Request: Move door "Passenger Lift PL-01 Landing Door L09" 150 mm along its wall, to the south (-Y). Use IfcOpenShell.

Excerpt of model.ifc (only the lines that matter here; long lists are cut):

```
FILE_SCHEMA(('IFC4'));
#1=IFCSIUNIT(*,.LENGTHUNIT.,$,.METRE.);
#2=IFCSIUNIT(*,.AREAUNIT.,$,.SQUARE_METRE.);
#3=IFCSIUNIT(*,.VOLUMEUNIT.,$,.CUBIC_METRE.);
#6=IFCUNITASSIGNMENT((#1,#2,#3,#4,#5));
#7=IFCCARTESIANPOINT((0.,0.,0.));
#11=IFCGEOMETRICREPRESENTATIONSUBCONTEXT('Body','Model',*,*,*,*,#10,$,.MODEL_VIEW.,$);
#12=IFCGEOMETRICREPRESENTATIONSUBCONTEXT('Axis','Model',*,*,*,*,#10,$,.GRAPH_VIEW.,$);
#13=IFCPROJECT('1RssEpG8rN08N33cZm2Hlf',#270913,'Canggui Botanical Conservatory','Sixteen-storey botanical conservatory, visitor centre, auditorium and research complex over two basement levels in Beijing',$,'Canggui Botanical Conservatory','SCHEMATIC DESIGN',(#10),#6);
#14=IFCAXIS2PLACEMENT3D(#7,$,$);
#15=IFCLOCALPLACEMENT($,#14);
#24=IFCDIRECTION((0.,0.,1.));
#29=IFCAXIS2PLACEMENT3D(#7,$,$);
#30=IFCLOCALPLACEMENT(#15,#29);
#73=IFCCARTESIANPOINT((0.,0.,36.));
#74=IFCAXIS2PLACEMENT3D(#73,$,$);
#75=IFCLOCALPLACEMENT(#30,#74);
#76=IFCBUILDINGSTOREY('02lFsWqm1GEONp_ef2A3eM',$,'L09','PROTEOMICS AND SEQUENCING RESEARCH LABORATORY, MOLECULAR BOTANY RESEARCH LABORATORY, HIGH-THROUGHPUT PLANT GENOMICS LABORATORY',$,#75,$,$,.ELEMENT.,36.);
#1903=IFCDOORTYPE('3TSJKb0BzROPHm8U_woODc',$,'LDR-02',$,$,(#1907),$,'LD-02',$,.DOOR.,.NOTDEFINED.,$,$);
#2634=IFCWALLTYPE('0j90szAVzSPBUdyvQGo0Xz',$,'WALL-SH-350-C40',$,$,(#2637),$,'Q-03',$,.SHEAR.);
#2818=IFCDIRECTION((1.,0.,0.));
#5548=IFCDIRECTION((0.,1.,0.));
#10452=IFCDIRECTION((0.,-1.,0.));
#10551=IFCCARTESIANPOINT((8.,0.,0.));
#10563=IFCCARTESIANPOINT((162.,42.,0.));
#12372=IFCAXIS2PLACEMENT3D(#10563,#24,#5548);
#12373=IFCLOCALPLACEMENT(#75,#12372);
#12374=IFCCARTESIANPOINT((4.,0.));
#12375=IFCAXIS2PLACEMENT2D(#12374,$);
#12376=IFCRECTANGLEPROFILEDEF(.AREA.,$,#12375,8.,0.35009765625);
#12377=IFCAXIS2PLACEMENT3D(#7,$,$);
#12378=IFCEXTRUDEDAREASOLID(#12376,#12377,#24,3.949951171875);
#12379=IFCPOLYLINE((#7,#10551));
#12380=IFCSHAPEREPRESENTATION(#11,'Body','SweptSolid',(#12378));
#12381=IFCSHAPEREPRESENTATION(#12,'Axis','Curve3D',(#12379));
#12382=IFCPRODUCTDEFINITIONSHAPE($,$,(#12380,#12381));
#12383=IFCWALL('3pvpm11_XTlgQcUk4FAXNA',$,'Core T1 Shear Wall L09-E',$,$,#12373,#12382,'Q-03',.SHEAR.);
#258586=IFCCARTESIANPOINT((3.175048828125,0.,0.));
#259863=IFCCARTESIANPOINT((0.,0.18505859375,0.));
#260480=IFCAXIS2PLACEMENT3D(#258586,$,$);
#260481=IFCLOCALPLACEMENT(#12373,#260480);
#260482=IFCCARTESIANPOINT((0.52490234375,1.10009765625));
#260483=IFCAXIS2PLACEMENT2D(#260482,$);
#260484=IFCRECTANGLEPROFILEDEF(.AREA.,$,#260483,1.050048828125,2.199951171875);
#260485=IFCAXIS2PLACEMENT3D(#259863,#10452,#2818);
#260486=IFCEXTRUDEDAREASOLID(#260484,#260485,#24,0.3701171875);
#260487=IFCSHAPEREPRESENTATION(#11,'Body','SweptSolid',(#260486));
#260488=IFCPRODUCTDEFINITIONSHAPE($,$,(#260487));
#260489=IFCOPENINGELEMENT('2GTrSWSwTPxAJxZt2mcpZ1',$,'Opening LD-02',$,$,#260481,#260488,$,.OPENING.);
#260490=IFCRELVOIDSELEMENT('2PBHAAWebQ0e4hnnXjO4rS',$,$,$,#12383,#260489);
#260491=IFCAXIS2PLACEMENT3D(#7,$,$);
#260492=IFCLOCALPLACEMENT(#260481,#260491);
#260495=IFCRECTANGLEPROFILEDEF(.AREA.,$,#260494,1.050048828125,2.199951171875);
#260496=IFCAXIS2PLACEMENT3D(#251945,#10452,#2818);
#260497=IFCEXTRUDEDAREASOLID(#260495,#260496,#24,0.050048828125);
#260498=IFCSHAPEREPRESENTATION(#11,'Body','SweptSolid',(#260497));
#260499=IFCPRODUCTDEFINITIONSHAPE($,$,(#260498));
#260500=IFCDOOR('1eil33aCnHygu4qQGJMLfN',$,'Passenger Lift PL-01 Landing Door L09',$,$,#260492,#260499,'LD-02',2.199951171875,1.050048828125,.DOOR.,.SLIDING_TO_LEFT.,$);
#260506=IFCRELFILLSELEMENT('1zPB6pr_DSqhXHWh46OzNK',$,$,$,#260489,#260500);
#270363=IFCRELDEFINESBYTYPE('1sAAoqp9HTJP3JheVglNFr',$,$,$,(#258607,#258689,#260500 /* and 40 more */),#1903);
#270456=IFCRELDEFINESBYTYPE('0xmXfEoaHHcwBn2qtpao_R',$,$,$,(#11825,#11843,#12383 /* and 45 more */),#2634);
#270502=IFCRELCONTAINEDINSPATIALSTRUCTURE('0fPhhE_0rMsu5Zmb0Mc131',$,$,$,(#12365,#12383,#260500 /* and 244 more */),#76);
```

```python
import ifcopenshell
import ifcopenshell.api.geometry
import ifcopenshell.util.placement
import ifcopenshell.util.unit

model = ifcopenshell.open("model.ifc")
unit_scale = ifcopenshell.util.unit.calculate_unit_scale(model)

door = model.by_id(260500)
opening = door.FillsVoids[0].RelatingOpeningElement
wall = opening.VoidsElements[0].RelatingBuildingElement

wall_matrix = ifcopenshell.util.placement.get_local_placement(wall.ObjectPlacement)
shift = wall_matrix[:3, 0] * -0.15 / unit_scale
before = ifcopenshell.util.placement.get_local_placement(door.ObjectPlacement)[:3, 3].copy()

# The door is placed relative to its opening, so it follows when the opening moves.
matrix = ifcopenshell.util.placement.get_local_placement(opening.ObjectPlacement)
matrix[:3, 3] += shift
ifcopenshell.api.geometry.edit_object_placement(
    model, product=opening, matrix=matrix, is_si=False, should_transform_children=True
)

after = ifcopenshell.util.placement.get_local_placement(door.ObjectPlacement)[:3, 3]
print("door moved by", (after - before).round(3) + 0.0)

model.write("model_updated.ifc")
```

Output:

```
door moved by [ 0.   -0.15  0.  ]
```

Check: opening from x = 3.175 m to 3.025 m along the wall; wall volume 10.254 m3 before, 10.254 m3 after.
